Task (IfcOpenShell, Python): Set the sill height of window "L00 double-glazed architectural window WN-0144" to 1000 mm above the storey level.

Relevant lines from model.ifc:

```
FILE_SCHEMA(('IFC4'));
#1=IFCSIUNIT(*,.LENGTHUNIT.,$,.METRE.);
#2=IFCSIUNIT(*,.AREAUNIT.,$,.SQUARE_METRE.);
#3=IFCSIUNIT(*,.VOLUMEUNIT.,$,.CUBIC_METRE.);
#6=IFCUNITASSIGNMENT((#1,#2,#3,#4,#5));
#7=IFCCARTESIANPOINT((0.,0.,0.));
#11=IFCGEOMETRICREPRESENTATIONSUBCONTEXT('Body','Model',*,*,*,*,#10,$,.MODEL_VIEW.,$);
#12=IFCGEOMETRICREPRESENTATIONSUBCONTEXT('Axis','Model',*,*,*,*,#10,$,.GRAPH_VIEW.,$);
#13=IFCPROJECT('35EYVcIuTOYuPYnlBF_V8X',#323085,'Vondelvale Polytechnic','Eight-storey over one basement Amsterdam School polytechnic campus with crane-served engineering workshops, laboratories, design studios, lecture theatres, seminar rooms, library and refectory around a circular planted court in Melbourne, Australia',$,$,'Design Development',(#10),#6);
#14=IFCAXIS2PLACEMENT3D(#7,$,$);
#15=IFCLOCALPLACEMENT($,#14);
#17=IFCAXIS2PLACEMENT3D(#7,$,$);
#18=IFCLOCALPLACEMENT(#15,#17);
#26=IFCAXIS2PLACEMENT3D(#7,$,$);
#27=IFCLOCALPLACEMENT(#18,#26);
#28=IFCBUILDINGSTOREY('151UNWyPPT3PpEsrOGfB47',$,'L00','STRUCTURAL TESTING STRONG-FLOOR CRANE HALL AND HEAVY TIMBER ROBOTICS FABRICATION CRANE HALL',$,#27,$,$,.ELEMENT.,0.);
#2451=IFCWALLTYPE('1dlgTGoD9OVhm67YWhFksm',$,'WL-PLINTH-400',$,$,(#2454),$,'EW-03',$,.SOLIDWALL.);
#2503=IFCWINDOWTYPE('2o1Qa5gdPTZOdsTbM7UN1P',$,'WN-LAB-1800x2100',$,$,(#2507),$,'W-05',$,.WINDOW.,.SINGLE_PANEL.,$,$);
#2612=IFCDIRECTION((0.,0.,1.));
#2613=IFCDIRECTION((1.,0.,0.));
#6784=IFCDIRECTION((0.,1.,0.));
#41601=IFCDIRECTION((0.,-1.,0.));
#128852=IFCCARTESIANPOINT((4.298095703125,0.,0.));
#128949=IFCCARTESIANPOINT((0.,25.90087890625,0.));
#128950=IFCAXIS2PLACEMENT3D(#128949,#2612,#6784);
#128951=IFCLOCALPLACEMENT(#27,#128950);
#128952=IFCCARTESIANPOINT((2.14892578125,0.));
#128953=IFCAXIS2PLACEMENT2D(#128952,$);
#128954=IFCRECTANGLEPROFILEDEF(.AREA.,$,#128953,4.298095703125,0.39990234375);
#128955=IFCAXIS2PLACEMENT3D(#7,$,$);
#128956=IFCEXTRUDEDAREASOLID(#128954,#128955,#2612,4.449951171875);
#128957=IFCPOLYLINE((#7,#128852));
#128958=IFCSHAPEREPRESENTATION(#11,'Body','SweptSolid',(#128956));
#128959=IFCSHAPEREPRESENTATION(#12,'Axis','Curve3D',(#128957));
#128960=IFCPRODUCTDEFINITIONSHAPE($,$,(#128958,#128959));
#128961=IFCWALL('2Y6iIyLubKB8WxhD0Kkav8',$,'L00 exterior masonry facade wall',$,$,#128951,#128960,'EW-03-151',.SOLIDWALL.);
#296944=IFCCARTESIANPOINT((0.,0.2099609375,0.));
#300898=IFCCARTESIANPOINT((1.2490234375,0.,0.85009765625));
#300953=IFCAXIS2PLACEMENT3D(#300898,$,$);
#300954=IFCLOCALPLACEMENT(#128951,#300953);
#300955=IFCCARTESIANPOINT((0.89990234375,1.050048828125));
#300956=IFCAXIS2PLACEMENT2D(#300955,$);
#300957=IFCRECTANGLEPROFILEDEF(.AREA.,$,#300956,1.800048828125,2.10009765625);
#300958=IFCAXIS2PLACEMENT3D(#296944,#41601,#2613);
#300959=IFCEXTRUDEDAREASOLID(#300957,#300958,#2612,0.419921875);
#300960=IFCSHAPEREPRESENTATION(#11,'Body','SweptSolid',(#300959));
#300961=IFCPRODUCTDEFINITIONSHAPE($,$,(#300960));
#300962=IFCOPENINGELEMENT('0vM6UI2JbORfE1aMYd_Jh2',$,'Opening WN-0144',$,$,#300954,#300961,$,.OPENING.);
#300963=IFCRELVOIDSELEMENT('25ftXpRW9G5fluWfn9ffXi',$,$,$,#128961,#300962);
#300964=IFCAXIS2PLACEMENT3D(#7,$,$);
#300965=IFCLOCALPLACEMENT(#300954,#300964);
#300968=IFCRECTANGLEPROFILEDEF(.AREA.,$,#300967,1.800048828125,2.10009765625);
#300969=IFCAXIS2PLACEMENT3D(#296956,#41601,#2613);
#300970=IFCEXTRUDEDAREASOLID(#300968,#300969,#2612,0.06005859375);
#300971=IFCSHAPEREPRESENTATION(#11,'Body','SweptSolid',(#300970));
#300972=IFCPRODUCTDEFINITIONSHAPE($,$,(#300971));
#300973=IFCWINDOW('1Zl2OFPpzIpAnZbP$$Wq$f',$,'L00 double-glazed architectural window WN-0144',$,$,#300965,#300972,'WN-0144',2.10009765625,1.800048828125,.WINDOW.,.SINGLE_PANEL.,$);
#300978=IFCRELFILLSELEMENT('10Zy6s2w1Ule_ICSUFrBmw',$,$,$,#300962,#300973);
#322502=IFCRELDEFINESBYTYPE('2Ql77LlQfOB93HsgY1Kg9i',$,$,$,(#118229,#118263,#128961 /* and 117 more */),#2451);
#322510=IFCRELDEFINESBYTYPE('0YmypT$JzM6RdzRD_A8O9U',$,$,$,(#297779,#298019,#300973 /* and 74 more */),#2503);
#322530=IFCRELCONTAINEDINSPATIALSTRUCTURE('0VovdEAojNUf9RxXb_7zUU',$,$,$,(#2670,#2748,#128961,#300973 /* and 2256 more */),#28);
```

```python
import numpy as np
import ifcopenshell
import ifcopenshell.api.geometry
import ifcopenshell.geom
import ifcopenshell.util.element
import ifcopenshell.util.placement
import ifcopenshell.util.shape
import ifcopenshell.util.unit

model = ifcopenshell.open("model.ifc")
unit_scale = ifcopenshell.util.unit.calculate_unit_scale(model)

window = model.by_guid("1Zl2OFPpzIpAnZbP$$Wq$f")
opening = window.FillsVoids[0].RelatingOpeningElement
storey = ifcopenshell.util.element.get_container(window, ifc_class="IfcBuildingStorey")
level = ifcopenshell.util.placement.get_local_placement(storey.ObjectPlacement)[2, 3]

# The opening's origin need not be at the sill, so measure its lowest point.
shape = ifcopenshell.geom.create_shape(ifcopenshell.geom.settings(), opening)
bottom = ifcopenshell.util.shape.get_shape_bottom_elevation(shape, shape.geometry) / unit_scale
dz = level + 1 / unit_scale - bottom

shift = np.array([0.0, 0.0, dz])
# The window is placed relative to its opening, so it follows when the opening moves.
matrix = ifcopenshell.util.placement.get_local_placement(opening.ObjectPlacement)
matrix[:3, 3] += shift
ifcopenshell.api.geometry.edit_object_placement(
    model, product=opening, matrix=matrix, is_si=False, should_transform_children=True
)

print(f"moved by {dz * unit_scale:+.3f} m")

model.write("model_v2.ifc")
```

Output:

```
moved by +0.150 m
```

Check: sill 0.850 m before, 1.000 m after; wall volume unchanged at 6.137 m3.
